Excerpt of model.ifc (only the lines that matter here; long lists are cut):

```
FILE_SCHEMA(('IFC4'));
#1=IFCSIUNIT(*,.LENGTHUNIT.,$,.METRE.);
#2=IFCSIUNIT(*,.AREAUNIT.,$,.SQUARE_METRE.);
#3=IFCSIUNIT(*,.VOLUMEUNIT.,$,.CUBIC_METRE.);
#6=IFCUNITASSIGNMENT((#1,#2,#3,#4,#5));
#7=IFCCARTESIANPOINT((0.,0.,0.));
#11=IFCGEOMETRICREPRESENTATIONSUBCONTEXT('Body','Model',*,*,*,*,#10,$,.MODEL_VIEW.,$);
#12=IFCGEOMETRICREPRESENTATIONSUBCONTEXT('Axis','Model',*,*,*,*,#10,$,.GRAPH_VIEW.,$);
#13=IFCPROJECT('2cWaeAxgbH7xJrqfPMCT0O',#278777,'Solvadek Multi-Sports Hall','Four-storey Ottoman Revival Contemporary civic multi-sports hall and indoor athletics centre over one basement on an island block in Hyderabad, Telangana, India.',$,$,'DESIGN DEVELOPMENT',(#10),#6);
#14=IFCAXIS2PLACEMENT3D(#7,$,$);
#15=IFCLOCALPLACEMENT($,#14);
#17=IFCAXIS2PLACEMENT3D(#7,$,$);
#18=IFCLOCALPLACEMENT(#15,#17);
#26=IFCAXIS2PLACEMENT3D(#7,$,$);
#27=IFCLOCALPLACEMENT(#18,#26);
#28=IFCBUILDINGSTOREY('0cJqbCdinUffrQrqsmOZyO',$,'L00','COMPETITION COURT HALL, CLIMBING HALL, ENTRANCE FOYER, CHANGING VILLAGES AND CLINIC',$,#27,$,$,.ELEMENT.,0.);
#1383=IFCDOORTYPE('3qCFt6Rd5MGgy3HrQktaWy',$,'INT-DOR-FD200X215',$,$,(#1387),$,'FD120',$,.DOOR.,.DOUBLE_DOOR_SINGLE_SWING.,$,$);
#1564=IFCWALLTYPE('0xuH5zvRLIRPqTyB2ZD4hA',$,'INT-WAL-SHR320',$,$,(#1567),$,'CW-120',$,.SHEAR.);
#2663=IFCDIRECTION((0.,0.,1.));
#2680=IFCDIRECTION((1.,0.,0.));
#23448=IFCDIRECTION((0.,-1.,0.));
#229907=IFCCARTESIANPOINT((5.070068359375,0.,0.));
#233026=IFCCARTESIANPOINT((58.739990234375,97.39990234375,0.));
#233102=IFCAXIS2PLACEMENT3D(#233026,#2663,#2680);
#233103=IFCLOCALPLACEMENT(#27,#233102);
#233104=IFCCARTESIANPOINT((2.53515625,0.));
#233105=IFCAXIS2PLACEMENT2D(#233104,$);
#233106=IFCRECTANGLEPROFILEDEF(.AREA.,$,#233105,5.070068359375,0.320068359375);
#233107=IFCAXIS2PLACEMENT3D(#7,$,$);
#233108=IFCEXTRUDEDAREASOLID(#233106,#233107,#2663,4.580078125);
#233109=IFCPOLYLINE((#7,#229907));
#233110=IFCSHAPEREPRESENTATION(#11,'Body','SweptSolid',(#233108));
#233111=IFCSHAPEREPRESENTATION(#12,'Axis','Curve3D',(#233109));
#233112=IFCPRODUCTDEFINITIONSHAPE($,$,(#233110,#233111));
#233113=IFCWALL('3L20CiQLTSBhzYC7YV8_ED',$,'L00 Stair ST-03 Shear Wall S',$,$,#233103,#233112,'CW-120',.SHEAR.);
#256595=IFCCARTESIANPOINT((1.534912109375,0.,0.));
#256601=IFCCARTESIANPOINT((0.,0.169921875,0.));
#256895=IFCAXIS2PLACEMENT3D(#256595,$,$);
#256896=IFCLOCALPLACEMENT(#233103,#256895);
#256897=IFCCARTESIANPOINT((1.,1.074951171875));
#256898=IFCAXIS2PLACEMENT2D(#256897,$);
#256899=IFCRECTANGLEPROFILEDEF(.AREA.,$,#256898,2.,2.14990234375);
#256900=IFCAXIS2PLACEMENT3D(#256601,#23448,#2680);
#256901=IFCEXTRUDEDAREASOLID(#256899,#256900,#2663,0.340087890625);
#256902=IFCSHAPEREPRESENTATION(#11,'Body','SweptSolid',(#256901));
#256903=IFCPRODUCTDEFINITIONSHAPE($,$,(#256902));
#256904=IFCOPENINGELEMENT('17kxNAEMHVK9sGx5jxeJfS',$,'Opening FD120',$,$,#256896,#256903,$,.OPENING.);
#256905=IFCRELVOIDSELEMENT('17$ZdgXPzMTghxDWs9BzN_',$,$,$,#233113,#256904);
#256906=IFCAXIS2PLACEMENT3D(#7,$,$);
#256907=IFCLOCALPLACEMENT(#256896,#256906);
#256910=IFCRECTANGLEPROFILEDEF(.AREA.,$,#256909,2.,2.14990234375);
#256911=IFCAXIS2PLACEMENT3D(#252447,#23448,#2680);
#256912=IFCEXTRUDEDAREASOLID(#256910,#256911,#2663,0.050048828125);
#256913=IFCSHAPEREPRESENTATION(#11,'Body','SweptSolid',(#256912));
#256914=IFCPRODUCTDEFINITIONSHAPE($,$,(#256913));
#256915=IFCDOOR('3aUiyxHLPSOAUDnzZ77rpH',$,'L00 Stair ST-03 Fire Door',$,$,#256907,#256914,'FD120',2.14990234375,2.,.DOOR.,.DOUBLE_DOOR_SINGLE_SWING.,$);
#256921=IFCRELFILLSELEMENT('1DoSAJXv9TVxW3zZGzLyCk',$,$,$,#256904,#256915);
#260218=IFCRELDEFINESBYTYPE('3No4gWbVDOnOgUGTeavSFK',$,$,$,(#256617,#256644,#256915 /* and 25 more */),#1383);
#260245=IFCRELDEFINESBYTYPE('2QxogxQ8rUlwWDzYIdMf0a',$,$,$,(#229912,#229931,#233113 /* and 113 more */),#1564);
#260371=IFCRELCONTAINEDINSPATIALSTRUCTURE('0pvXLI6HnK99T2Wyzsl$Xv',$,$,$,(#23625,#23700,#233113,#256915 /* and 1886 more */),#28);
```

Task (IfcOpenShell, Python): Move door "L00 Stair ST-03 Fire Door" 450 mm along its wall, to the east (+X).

```python
import ifcopenshell
import ifcopenshell.api.geometry
import ifcopenshell.util.placement
import ifcopenshell.util.unit

model = ifcopenshell.open("model.ifc")
unit_scale = ifcopenshell.util.unit.calculate_unit_scale(model)

door = model.by_guid("3aUiyxHLPSOAUDnzZ77rpH")
opening = door.FillsVoids[0].RelatingOpeningElement
wall = opening.VoidsElements[0].RelatingBuildingElement

wall_matrix = ifcopenshell.util.placement.get_local_placement(wall.ObjectPlacement)
shift = wall_matrix[:3, 0] * 0.45 / unit_scale
before = ifcopenshell.util.placement.get_local_placement(door.ObjectPlacement)[:3, 3].copy()

# The door is placed relative to its opening, so it follows when the opening moves.
matrix = ifcopenshell.util.placement.get_local_placement(opening.ObjectPlacement)
matrix[:3, 3] += shift
ifcopenshell.api.geometry.edit_object_placement(
    model, product=opening, matrix=matrix, is_si=False, should_transform_children=True
)

after = ifcopenshell.util.placement.get_local_placement(door.ObjectPlacement)[:3, 3]
print("door moved by", (after - before).round(3) + 0.0)

model.write("model_rev.ifc")
```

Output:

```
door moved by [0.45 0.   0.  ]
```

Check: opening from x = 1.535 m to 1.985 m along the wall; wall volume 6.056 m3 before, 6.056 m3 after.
